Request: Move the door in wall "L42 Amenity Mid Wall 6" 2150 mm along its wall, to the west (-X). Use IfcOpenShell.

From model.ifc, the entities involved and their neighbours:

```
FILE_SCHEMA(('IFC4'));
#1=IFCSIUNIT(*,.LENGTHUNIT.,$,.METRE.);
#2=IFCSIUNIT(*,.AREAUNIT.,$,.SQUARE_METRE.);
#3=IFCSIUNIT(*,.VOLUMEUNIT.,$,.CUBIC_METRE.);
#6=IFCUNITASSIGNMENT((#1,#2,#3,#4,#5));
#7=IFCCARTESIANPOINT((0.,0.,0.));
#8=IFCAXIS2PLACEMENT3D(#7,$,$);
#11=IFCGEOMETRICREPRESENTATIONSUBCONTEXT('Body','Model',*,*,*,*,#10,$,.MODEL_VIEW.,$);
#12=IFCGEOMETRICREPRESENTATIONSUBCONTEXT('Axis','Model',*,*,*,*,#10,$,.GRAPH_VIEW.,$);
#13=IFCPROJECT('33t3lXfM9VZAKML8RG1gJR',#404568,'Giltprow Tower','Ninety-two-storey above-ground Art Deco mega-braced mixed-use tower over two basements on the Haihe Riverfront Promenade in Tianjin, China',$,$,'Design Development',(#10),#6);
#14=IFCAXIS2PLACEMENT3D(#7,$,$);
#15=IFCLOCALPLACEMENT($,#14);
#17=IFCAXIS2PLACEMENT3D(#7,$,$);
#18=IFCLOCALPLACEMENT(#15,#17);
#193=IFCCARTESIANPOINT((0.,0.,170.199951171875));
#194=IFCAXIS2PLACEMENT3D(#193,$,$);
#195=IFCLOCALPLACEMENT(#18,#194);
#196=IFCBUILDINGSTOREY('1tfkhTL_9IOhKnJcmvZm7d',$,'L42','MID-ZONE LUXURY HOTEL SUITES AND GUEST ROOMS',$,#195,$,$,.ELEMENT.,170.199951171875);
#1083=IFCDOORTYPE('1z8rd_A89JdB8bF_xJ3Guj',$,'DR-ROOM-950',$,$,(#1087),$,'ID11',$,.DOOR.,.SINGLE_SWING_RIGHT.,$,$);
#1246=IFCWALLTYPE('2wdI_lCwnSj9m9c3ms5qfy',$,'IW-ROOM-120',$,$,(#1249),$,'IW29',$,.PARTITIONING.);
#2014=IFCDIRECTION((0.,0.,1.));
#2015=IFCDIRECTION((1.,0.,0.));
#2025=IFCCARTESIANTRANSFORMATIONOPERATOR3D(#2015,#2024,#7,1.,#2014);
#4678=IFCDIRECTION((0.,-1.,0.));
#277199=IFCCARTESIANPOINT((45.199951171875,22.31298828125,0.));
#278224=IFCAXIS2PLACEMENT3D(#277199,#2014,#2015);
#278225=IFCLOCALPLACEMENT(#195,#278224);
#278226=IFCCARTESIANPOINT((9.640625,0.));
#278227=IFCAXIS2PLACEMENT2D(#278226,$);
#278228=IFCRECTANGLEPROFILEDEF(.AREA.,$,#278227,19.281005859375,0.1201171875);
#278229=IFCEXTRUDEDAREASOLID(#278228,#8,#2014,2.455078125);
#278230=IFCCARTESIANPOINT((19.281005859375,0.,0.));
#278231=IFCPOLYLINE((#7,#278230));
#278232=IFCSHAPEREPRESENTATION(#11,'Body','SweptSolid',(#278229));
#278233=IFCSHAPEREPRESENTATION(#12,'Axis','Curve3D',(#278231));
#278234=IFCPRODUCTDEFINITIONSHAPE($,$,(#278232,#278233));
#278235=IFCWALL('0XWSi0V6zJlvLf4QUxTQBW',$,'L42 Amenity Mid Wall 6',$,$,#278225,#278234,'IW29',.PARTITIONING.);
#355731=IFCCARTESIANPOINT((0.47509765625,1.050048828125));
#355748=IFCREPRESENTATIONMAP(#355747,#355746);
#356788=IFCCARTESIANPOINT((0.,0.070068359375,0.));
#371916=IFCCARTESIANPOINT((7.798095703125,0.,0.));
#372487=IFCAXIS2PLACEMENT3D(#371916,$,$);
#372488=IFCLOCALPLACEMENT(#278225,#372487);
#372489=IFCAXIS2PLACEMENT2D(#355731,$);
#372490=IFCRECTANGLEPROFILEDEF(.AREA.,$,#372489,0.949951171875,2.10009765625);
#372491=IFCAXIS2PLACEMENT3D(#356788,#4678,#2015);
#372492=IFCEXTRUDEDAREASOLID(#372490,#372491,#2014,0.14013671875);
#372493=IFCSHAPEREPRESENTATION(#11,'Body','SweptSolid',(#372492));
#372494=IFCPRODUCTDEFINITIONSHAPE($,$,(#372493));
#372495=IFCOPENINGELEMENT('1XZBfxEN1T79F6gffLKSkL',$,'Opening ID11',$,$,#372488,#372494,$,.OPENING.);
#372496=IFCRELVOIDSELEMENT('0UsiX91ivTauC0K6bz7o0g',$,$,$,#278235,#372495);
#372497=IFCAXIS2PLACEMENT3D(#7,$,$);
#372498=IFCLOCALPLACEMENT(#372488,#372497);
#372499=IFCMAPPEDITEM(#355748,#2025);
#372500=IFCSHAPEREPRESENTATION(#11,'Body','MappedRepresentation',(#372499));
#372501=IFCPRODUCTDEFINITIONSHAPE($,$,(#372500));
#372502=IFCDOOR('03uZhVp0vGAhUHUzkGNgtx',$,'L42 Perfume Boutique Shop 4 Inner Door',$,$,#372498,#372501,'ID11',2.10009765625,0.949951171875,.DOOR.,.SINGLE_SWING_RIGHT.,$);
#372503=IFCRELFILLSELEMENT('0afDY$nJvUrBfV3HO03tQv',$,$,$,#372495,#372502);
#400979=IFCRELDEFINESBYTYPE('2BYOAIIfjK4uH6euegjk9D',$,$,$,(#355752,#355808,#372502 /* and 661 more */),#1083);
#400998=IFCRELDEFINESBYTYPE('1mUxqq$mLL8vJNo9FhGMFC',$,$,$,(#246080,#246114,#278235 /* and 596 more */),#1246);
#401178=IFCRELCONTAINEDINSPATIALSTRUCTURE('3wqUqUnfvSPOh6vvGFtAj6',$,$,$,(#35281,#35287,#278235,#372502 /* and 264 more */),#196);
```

```python
import ifcopenshell
import ifcopenshell.api.geometry
import ifcopenshell.util.placement
import ifcopenshell.util.unit

model = ifcopenshell.open("model.ifc")
unit_scale = ifcopenshell.util.unit.calculate_unit_scale(model)

door = model.by_guid("03uZhVp0vGAhUHUzkGNgtx")
opening = door.FillsVoids[0].RelatingOpeningElement
wall = opening.VoidsElements[0].RelatingBuildingElement

wall_matrix = ifcopenshell.util.placement.get_local_placement(wall.ObjectPlacement)
shift = wall_matrix[:3, 0] * -2.15 / unit_scale
before = ifcopenshell.util.placement.get_local_placement(door.ObjectPlacement)[:3, 3].copy()

# The door is placed relative to its opening, so it follows when the opening moves.
matrix = ifcopenshell.util.placement.get_local_placement(opening.ObjectPlacement)
matrix[:3, 3] += shift
ifcopenshell.api.geometry.edit_object_placement(
    model, product=opening, matrix=matrix, is_si=False, should_transform_children=True
)

after = ifcopenshell.util.placement.get_local_placement(door.ObjectPlacement)[:3, 3]
print("door moved by", (after - before).round(3) + 0.0)

model.write("model-out.ifc")
```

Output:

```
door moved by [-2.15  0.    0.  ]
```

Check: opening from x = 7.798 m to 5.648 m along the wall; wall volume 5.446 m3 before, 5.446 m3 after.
